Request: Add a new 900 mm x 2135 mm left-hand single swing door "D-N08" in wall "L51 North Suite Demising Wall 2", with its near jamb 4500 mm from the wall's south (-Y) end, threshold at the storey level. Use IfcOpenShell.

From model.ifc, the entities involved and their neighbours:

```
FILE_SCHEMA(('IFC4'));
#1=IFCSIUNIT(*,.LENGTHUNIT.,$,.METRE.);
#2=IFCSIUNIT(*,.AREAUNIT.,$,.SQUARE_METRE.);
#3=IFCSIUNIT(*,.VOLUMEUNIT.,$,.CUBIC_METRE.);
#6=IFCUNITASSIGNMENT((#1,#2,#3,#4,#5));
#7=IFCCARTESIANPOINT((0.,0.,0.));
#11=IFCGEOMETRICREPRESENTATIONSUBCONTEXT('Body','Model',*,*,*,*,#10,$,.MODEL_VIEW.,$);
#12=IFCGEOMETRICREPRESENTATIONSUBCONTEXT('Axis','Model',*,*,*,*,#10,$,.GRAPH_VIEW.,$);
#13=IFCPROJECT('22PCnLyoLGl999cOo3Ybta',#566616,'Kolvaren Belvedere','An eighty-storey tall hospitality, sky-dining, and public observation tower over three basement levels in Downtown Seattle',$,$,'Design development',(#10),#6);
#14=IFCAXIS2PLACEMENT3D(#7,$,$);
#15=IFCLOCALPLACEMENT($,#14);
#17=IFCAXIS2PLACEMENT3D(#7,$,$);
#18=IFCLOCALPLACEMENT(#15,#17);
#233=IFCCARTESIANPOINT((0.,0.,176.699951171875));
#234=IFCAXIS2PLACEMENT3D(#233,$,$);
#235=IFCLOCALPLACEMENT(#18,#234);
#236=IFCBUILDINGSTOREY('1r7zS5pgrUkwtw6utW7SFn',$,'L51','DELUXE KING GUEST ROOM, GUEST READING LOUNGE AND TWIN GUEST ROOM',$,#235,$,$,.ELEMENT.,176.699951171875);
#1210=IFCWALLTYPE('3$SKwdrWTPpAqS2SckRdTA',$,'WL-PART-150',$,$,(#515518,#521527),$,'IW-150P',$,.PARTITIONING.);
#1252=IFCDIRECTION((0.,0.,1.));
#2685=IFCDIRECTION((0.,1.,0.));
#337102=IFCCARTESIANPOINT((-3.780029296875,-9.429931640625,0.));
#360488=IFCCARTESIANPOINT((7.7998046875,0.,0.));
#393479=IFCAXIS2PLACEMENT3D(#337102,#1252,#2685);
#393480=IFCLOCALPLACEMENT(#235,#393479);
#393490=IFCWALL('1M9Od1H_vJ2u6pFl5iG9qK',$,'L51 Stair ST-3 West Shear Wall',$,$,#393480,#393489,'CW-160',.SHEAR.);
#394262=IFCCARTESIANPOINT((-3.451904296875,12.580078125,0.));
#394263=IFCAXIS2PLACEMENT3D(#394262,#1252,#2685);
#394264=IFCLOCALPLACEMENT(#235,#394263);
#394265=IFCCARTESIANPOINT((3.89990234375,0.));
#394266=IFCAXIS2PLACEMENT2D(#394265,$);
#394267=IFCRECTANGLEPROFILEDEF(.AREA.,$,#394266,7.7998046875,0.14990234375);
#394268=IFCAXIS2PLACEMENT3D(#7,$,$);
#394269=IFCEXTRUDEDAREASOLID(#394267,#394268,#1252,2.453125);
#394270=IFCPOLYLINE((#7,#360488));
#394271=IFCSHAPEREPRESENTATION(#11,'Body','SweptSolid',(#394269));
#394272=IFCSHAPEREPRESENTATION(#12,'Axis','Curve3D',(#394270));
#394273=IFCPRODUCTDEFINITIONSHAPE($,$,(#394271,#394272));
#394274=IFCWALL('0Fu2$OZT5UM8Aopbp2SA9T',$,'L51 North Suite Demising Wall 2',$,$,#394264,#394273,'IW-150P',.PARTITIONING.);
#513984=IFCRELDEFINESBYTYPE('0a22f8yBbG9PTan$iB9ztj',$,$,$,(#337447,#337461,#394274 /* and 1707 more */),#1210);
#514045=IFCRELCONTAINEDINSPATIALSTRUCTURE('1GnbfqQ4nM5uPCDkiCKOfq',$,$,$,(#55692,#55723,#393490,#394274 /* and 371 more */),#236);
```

```python
import numpy as np
import ifcopenshell
import ifcopenshell.api.feature
import ifcopenshell.api.geometry
import ifcopenshell.api.root
import ifcopenshell.api.spatial
import ifcopenshell.geom
import ifcopenshell.util.element
import ifcopenshell.util.placement
import ifcopenshell.util.representation
import ifcopenshell.util.shape
import ifcopenshell.util.unit

model = ifcopenshell.open("model.ifc")
unit_scale = ifcopenshell.util.unit.calculate_unit_scale(model)
settings = ifcopenshell.geom.settings()


def volume(element):
    """Net volume in cubic metres, openings subtracted."""
    shape = ifcopenshell.geom.create_shape(settings, element)
    return ifcopenshell.util.shape.get_volume(shape.geometry)


wall = model.by_guid("0Fu2$OZT5UM8Aopbp2SA9T")
storey = ifcopenshell.util.element.get_container(wall, ifc_class="IfcBuildingStorey")
context = ifcopenshell.util.representation.get_context(model, "Model", "Body", "MODEL_VIEW")
before = volume(wall)

width, height, from_end, sill = 0.9, 2.135, 4.5, 0.0  # metres

# The wall runs along its own X axis, and the end named is its -X end.
wall_shape = ifcopenshell.geom.create_shape(settings, wall)
x, y, z = ifcopenshell.util.shape.get_vertices(wall_shape.geometry).T
start = x.min() + from_end
face, thickness = float(y.min()), float(y.max() - y.min())
wall_matrix = ifcopenshell.util.placement.get_local_placement(wall.ObjectPlacement)
level = ifcopenshell.util.placement.get_local_placement(storey.ObjectPlacement)[2, 3]


def in_wall(x, y):
    """Placement at x, y metres in the wall's axes, at sill height."""
    matrix = wall_matrix.copy()
    matrix[:, 3] = wall_matrix @ np.array([x / unit_scale, y / unit_scale, 0.0, 1.0])
    matrix[2, 3] = level + sill / unit_scale
    return matrix


# Opening: a box that overshoots both wall faces by 50 mm.
opening = ifcopenshell.api.root.create_entity(model, ifc_class="IfcOpeningElement", predefined_type="OPENING")
box = ifcopenshell.api.geometry.add_wall_representation(
    model, context=context, length=width, height=height, thickness=thickness + 0.1
)
ifcopenshell.api.geometry.assign_representation(model, product=opening, representation=box)
ifcopenshell.api.geometry.edit_object_placement(model, product=opening, matrix=in_wall(start, face - 0.05), is_si=False)
ifcopenshell.api.feature.add_feature(model, feature=opening, element=wall)

door = ifcopenshell.api.root.create_entity(model, ifc_class="IfcDoor", name="D-N08", predefined_type="DOOR")
door.OverallWidth, door.OverallHeight = width / unit_scale, height / unit_scale
door.OperationType = "SINGLE_SWING_LEFT"
body = ifcopenshell.api.geometry.add_door_representation(
    model,
    context=context,
    overall_width=door.OverallWidth,
    overall_height=door.OverallHeight,
    operation_type="SINGLE_SWING_LEFT",
    lining_properties={"LiningDepth": thickness / unit_scale, "ThresholdDepth": thickness / unit_scale},
)
ifcopenshell.api.geometry.assign_representation(model, product=door, representation=body)
ifcopenshell.api.spatial.assign_container(model, products=[door], relating_structure=storey)
ifcopenshell.api.feature.add_filling(model, opening=opening, element=door)

# The lining spans the wall, so the door starts at the wall face.
ifcopenshell.api.geometry.edit_object_placement(model, product=door, matrix=in_wall(start, face), is_si=False)

after = volume(wall)

print(f"wall volume {before:.3f} -> {after:.3f} m3")

model.write("model-out.ifc")
```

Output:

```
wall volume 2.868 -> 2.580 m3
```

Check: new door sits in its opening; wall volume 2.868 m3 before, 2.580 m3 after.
